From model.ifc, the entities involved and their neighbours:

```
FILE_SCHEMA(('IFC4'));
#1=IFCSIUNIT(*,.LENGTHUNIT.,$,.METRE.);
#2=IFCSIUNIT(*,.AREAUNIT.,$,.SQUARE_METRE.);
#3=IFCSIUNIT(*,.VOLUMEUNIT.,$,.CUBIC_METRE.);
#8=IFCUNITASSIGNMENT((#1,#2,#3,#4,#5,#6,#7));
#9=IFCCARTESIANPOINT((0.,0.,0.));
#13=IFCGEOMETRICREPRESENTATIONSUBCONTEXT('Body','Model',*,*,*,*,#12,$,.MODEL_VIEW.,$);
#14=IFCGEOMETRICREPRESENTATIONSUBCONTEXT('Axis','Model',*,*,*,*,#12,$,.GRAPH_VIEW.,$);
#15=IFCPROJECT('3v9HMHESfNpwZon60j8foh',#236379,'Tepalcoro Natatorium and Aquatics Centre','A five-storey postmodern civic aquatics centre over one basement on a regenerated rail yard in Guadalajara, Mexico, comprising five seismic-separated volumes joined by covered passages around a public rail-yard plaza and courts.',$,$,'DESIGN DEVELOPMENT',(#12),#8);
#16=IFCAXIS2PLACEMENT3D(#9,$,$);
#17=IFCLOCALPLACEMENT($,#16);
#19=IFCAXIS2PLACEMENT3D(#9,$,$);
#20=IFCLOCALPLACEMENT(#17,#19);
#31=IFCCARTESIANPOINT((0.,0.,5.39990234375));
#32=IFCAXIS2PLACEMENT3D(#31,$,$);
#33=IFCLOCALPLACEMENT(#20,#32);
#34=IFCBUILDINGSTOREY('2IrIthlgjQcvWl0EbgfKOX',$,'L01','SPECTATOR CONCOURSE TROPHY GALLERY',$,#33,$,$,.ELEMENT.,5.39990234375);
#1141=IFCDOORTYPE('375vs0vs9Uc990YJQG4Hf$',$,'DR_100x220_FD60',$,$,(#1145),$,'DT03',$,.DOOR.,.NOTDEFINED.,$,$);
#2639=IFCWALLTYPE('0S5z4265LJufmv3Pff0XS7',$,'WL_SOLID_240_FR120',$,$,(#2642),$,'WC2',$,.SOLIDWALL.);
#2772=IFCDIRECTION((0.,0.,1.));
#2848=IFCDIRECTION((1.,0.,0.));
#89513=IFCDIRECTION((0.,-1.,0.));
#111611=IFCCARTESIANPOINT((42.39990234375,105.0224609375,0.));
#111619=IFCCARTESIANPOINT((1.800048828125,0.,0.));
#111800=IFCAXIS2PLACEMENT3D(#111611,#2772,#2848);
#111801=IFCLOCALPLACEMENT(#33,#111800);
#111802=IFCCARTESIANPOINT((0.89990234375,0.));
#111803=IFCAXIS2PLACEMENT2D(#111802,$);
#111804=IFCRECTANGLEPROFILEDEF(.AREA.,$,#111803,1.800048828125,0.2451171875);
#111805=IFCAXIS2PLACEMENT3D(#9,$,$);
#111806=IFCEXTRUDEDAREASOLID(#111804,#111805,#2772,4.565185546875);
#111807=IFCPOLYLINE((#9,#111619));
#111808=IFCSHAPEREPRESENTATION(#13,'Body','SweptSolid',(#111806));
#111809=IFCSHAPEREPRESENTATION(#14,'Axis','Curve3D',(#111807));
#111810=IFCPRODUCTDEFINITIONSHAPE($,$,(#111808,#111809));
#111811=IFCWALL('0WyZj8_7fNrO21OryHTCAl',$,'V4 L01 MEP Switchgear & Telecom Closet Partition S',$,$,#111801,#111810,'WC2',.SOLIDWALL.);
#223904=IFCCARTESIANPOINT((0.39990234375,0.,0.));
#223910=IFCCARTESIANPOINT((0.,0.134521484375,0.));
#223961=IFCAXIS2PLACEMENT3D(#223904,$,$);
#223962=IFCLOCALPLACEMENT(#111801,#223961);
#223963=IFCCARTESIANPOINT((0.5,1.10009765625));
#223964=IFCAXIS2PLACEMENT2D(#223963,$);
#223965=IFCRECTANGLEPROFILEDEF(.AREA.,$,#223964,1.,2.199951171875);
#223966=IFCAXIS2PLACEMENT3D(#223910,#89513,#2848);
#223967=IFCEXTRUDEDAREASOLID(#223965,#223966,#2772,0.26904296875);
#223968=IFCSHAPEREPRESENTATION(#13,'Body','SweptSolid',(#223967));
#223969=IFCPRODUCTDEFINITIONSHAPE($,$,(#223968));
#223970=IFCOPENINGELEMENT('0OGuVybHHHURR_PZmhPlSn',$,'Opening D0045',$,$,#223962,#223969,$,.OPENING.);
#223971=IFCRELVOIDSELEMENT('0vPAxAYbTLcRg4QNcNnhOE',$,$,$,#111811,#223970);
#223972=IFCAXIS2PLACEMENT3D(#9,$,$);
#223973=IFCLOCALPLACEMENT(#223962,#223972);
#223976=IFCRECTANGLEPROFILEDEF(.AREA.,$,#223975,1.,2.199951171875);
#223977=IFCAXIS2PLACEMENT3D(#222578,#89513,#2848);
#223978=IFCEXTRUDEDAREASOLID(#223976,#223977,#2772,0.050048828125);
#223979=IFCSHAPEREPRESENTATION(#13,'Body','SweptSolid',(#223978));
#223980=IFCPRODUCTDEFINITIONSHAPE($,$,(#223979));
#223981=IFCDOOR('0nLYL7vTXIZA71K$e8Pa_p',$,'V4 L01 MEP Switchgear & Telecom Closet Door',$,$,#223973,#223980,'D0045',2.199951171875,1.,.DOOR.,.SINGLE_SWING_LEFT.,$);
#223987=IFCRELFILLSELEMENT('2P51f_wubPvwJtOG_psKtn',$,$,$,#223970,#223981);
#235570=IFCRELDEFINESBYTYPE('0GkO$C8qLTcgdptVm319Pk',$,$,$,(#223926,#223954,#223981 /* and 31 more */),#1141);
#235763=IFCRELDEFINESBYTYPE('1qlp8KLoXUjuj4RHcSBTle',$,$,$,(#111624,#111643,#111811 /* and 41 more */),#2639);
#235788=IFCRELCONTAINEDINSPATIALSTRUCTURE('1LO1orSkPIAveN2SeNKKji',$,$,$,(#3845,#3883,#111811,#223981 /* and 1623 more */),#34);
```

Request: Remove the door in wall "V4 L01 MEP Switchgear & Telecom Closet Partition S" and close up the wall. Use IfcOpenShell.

```python
import ifcopenshell
import ifcopenshell.api.feature
import ifcopenshell.api.root
import ifcopenshell.geom
import ifcopenshell.util.shape

model = ifcopenshell.open("model.ifc")
settings = ifcopenshell.geom.settings()


def volume(element):
    """Net volume in cubic metres, openings subtracted."""
    shape = ifcopenshell.geom.create_shape(settings, element)
    return ifcopenshell.util.shape.get_volume(shape.geometry)


door = model.by_id(223981)
opening = door.FillsVoids[0].RelatingOpeningElement
wall = opening.VoidsElements[0].RelatingBuildingElement
before = volume(wall)

ifcopenshell.api.root.remove_product(model, product=door)
ifcopenshell.api.feature.remove_feature(model, feature=opening)

after = volume(wall)

print(f"wall volume {before:.3f} -> {after:.3f} m3")

model.write("model_v2.ifc")
```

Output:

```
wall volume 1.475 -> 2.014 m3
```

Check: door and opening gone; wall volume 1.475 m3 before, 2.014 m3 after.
